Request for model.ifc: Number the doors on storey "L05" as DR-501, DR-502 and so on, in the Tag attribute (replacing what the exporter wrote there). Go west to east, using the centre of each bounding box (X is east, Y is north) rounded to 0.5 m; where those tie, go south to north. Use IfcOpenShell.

First a look at what the model holds.

```python
import ifcopenshell
import ifcopenshell.util.element
import ifcopenshell.util.placement

model = ifcopenshell.open("model.ifc")
print(model.schema)
storey = next(s for s in model.by_type("IfcBuildingStorey") if s.Name == "L05")
doors = [e for e in ifcopenshell.util.element.get_decomposition(storey) if e.is_a("IfcDoor")]
for e in sorted(doors, key=lambda e: e.id()):
    origin = ifcopenshell.util.placement.get_local_placement(e.ObjectPlacement)[:3, 3]
    print(e.id(), e.Tag, e.Name, origin.round(2) + 0.0, sep=" | ")
```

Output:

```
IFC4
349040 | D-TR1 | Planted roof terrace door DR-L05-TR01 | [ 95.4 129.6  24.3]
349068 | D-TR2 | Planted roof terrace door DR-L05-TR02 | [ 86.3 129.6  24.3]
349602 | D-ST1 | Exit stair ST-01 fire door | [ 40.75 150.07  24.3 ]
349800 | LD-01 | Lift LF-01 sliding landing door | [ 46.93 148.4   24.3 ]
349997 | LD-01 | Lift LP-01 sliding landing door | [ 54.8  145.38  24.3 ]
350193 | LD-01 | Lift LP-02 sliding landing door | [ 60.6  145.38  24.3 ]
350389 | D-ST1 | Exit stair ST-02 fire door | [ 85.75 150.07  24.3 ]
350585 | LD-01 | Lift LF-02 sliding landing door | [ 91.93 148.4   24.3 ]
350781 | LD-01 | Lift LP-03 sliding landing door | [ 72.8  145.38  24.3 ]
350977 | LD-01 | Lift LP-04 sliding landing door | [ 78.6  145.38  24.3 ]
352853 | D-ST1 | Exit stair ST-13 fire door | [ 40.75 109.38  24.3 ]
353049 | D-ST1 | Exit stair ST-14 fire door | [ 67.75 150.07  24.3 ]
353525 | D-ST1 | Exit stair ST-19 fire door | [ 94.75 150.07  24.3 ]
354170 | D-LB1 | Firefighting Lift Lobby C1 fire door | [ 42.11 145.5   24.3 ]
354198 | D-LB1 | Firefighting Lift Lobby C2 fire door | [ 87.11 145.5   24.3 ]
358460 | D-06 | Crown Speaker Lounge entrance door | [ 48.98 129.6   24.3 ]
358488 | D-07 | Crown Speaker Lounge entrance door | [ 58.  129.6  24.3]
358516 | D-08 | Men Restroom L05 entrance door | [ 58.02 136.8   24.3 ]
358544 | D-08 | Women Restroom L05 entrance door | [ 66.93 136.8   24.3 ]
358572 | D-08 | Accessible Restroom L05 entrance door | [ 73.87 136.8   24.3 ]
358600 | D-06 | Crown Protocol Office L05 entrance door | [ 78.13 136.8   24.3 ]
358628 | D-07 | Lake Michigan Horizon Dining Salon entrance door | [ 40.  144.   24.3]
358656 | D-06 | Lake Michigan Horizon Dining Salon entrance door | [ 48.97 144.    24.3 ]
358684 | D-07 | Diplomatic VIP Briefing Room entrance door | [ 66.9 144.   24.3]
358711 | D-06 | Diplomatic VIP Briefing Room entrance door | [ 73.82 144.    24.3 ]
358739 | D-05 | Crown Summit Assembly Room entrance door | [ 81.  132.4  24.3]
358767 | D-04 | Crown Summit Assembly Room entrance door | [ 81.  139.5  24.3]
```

```python
import ifcopenshell
import ifcopenshell.geom
import ifcopenshell.util.element
import ifcopenshell.util.shape

model = ifcopenshell.open("model.ifc")
settings = ifcopenshell.geom.settings()
settings.set("use-world-coords", True)


def centre(element):
    shape = ifcopenshell.geom.create_shape(settings, element)
    return ifcopenshell.util.shape.get_bbox_centroid(shape.geometry)


storey = next(s for s in model.by_type("IfcBuildingStorey") if s.Name == "L05")
doors = [e for e in ifcopenshell.util.element.get_decomposition(storey) if e.is_a("IfcDoor")]

# Insertion points can sit at a corner or the storey origin, so sort by the geometry (in metres).
centres = {e: centre(e) for e in doors}
doors.sort(key=lambda e: (round(centres[e][0] / 0.5), centres[e][1]))

for i, e in enumerate(doors, start=1):
    number = f"DR-5{i:02d}"
    e.Tag = number
    print(e.id(), number)

model.write("model_edited.ifc")
```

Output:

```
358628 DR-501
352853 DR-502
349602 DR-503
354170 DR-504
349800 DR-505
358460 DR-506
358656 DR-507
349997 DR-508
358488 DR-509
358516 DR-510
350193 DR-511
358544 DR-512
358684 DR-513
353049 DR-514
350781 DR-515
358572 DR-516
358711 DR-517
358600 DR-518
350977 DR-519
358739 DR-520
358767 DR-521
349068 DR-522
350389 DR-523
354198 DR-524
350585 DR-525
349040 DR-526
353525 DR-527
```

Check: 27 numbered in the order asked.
